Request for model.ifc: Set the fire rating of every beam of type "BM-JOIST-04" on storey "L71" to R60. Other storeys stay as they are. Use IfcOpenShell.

First a look at what the model holds.

```python
import ifcopenshell
import ifcopenshell.util.element

model = ifcopenshell.open("model.ifc")
print(model.schema)
storey = next(s for s in model.by_type("IfcBuildingStorey") if s.Name == "L71")
beams = [e for e in ifcopenshell.util.element.get_decomposition(storey) if e.is_a("IfcBeam")]
seen = {}
for e in beams:
    element_type = ifcopenshell.util.element.get_type(e)
    key = (element_type.Name if element_type != e and element_type else None, ifcopenshell.util.element.get_pset(e, "Pset_BeamCommon", "FireRating"))
    seen[key] = seen.get(key, 0) + 1
for (name, value), count in sorted(seen.items(), key=str):
    print(count, "x", name, "|", value)
```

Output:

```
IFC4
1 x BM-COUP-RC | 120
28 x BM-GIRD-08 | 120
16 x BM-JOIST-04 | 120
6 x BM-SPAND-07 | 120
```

```python
import ifcopenshell
import ifcopenshell.api.pset
import ifcopenshell.util.element

model = ifcopenshell.open("model.ifc")

storey = next(s for s in model.by_type("IfcBuildingStorey") if s.Name == "L71")
beams = [e for e in ifcopenshell.util.element.get_decomposition(storey) if e.is_a("IfcBeam")]

count = 0
for e in beams:
    element_type = ifcopenshell.util.element.get_type(e)
    if element_type in (None, e) or element_type.Name != "BM-JOIST-04":
        continue
    # add_pset returns the element's existing set when there is one.
    pset = ifcopenshell.api.pset.add_pset(model, product=e, name="Pset_BeamCommon")
    ifcopenshell.api.pset.edit_pset(model, pset=pset, properties={"FireRating": "R60"})
    count += 1

print(count, "beams updated")

model.write("model_rev.ifc")
```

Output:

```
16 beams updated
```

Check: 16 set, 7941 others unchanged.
